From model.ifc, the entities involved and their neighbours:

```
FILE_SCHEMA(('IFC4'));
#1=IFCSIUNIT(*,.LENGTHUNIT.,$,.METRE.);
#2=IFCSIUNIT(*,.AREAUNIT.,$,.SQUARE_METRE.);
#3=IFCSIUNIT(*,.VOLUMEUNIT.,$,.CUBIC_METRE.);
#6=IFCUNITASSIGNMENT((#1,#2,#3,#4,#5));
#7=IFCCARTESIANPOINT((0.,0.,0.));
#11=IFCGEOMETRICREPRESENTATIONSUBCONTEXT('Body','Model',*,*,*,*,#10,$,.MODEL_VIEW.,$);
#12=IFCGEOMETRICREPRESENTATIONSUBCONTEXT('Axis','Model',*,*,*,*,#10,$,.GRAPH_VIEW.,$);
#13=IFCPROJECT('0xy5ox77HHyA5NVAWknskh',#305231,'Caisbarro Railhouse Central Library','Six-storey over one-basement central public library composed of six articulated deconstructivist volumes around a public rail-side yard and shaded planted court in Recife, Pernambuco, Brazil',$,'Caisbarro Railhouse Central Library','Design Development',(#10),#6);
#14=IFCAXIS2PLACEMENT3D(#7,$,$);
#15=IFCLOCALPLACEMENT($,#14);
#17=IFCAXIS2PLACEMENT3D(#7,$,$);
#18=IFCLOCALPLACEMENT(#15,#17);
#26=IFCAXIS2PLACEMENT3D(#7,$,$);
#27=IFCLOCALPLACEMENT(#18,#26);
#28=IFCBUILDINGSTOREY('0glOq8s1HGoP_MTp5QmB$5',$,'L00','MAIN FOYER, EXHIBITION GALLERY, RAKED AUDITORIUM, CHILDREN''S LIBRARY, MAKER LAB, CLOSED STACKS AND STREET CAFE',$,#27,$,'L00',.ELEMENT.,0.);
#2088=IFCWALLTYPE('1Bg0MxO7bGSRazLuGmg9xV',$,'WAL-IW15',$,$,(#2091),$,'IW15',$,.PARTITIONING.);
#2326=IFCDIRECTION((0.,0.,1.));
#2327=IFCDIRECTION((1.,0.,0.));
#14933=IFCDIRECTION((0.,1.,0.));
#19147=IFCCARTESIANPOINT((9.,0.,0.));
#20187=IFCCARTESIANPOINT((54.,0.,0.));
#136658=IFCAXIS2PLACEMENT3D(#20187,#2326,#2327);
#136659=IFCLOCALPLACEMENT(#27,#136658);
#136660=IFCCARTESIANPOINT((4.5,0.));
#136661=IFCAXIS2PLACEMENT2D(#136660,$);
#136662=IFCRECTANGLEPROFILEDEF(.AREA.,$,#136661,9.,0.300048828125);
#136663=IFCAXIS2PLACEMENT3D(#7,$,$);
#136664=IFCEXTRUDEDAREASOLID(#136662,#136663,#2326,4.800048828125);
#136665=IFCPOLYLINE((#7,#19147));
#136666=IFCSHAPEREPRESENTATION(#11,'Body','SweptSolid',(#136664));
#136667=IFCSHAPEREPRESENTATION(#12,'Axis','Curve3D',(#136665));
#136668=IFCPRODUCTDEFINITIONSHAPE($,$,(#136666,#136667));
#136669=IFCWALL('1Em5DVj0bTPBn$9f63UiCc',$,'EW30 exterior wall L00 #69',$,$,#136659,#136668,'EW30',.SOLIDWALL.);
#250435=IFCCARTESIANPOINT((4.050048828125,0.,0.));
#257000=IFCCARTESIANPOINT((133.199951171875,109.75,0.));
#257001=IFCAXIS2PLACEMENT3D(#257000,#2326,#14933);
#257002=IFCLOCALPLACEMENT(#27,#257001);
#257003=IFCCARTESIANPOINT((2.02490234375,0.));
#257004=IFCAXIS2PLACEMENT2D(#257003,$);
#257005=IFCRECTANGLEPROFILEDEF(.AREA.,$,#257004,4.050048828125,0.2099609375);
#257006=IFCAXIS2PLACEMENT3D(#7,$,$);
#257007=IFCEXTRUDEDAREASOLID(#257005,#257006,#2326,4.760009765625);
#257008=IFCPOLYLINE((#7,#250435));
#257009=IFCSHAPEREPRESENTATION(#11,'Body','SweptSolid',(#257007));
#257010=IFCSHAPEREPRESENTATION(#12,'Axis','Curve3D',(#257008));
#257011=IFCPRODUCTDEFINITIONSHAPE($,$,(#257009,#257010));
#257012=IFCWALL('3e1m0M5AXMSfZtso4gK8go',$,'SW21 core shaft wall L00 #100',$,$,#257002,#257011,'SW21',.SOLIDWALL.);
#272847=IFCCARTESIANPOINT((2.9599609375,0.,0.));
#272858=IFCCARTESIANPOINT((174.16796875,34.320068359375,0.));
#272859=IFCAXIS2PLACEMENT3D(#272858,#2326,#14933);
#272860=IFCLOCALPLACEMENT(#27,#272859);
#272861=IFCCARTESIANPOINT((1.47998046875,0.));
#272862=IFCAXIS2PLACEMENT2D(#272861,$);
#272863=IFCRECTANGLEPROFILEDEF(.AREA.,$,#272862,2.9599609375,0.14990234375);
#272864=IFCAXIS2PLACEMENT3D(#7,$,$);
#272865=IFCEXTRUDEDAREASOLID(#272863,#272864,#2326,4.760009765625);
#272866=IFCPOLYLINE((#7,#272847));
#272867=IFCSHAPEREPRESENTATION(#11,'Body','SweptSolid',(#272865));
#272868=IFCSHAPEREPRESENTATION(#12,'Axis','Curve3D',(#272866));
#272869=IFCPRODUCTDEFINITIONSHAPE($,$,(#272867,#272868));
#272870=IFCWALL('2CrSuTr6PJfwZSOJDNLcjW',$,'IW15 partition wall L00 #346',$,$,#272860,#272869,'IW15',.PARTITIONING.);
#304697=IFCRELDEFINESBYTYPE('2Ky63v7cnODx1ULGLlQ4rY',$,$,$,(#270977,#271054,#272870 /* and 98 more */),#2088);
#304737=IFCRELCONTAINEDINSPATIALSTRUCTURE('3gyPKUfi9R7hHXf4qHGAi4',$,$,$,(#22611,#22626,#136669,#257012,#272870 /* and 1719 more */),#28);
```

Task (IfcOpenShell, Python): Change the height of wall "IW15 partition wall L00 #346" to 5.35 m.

```python
import ifcopenshell
import ifcopenshell.geom
import ifcopenshell.util.representation
import ifcopenshell.util.shape
import ifcopenshell.util.unit

model = ifcopenshell.open("model.ifc")
unit_scale = ifcopenshell.util.unit.calculate_unit_scale(model)
settings = ifcopenshell.geom.settings()


def volume(element):
    """Net volume in cubic metres, openings subtracted."""
    shape = ifcopenshell.geom.create_shape(settings, element)
    return ifcopenshell.util.shape.get_volume(shape.geometry)


wall = model.by_guid("2CrSuTr6PJfwZSOJDNLcjW")
before = volume(wall)

body = ifcopenshell.util.representation.get_representation(wall, "Model", "Body")
solid = body.Items[0]
old_height = solid.Depth
solid.Depth = 5.35 / unit_scale
after = volume(wall)

print(f"height {old_height:g} -> {solid.Depth:g}, volume {before:.3f} -> {after:.3f} m3")

model.write("model_rev.ifc")
```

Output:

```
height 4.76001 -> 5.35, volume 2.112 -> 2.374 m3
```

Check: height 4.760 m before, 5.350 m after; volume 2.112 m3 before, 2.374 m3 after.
